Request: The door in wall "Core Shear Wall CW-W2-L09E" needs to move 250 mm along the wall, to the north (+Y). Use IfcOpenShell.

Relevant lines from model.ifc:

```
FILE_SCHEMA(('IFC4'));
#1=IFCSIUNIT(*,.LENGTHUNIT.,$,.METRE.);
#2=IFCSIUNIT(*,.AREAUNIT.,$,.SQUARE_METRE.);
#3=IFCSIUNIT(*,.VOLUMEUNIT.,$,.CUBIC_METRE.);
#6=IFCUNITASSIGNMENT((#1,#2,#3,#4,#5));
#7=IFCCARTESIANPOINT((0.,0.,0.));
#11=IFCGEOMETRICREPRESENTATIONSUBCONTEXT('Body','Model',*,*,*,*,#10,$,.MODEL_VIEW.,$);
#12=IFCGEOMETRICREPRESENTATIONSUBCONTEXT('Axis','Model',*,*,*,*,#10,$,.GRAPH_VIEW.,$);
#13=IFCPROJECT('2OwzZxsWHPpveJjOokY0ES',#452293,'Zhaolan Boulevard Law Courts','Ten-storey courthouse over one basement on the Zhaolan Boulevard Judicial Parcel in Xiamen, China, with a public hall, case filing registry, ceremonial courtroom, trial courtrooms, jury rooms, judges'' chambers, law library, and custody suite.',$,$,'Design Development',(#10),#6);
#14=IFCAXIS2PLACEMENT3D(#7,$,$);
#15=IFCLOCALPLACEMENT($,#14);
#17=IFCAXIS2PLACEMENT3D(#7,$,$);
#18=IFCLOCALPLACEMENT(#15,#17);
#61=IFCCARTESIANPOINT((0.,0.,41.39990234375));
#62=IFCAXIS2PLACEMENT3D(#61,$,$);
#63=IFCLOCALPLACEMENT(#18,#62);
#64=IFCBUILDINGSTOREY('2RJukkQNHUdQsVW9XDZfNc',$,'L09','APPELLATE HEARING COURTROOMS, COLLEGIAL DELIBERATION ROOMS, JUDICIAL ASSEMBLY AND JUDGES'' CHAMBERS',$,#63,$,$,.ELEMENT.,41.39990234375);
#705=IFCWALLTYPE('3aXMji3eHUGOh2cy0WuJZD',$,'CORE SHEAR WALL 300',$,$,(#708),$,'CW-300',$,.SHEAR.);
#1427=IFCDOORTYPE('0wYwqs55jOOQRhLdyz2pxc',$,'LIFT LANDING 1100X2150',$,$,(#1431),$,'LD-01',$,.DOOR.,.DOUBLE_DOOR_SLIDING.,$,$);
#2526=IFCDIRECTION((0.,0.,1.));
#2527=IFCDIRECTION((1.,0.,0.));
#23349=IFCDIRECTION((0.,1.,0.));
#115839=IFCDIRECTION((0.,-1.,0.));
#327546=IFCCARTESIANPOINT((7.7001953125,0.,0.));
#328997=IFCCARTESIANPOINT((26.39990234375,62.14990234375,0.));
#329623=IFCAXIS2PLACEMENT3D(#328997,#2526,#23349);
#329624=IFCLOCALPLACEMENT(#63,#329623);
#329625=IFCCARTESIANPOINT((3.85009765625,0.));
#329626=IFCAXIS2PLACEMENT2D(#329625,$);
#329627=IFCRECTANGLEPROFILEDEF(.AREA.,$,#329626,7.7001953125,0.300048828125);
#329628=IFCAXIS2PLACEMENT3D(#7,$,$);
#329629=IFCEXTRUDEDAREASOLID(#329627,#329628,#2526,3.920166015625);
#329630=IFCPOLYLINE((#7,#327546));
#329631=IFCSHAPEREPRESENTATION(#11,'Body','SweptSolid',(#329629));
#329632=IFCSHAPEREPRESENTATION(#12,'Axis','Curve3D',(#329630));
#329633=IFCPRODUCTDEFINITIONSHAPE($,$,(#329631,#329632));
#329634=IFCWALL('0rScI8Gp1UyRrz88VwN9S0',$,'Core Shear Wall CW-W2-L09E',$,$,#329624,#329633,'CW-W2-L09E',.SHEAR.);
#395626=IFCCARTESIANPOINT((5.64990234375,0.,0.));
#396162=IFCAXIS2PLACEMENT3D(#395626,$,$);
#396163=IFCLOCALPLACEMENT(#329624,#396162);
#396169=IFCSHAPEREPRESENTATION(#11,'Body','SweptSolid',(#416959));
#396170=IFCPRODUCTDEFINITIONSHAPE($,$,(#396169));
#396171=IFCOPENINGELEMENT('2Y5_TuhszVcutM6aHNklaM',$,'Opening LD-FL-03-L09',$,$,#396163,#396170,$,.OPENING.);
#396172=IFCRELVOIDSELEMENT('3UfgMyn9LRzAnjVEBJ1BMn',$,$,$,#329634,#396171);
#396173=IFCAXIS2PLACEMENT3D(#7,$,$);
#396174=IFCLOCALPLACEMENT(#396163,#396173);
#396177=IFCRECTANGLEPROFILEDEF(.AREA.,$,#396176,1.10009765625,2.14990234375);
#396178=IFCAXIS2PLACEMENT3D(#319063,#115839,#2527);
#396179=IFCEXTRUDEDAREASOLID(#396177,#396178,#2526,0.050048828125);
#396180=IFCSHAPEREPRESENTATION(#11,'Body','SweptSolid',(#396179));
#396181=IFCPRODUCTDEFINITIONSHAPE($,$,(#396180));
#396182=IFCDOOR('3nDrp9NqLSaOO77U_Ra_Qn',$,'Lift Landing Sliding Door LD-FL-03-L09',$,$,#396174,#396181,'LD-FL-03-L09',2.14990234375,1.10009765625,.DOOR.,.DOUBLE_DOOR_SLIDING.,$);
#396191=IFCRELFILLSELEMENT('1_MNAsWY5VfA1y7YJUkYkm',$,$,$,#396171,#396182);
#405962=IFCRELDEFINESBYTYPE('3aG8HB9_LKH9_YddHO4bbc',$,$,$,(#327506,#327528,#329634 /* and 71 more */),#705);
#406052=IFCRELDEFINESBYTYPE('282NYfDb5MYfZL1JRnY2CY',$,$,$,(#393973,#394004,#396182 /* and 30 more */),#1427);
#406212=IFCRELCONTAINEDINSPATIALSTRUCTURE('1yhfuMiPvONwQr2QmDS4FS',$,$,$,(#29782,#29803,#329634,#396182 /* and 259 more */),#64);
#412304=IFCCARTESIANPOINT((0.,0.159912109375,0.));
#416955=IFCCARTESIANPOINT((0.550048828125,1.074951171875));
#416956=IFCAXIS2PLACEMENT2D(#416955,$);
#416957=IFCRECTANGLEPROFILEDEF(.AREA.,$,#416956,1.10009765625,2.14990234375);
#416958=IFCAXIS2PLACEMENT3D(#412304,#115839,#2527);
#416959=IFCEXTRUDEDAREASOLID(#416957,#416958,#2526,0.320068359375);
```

```python
import ifcopenshell
import ifcopenshell.api.geometry
import ifcopenshell.util.placement

model = ifcopenshell.open("model.ifc")

door = model.by_guid("3nDrp9NqLSaOO77U_Ra_Qn")
opening = door.FillsVoids[0].RelatingOpeningElement
wall = opening.VoidsElements[0].RelatingBuildingElement

wall_matrix = ifcopenshell.util.placement.get_local_placement(wall.ObjectPlacement)
shift = wall_matrix[:3, 0] * 0.25
before = ifcopenshell.util.placement.get_local_placement(door.ObjectPlacement)[:3, 3].copy()

# The door is placed relative to its opening, so it follows when the opening moves.
matrix = ifcopenshell.util.placement.get_local_placement(opening.ObjectPlacement)
matrix[:3, 3] += shift
ifcopenshell.api.geometry.edit_object_placement(
    model, product=opening, matrix=matrix, is_si=False, should_transform_children=True
)

after = ifcopenshell.util.placement.get_local_placement(door.ObjectPlacement)[:3, 3]
print("door moved by", (after - before).round(3) + 0.0)

model.write("model-out.ifc")
```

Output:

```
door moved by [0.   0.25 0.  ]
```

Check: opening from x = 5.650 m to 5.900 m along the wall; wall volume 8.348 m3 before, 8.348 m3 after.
